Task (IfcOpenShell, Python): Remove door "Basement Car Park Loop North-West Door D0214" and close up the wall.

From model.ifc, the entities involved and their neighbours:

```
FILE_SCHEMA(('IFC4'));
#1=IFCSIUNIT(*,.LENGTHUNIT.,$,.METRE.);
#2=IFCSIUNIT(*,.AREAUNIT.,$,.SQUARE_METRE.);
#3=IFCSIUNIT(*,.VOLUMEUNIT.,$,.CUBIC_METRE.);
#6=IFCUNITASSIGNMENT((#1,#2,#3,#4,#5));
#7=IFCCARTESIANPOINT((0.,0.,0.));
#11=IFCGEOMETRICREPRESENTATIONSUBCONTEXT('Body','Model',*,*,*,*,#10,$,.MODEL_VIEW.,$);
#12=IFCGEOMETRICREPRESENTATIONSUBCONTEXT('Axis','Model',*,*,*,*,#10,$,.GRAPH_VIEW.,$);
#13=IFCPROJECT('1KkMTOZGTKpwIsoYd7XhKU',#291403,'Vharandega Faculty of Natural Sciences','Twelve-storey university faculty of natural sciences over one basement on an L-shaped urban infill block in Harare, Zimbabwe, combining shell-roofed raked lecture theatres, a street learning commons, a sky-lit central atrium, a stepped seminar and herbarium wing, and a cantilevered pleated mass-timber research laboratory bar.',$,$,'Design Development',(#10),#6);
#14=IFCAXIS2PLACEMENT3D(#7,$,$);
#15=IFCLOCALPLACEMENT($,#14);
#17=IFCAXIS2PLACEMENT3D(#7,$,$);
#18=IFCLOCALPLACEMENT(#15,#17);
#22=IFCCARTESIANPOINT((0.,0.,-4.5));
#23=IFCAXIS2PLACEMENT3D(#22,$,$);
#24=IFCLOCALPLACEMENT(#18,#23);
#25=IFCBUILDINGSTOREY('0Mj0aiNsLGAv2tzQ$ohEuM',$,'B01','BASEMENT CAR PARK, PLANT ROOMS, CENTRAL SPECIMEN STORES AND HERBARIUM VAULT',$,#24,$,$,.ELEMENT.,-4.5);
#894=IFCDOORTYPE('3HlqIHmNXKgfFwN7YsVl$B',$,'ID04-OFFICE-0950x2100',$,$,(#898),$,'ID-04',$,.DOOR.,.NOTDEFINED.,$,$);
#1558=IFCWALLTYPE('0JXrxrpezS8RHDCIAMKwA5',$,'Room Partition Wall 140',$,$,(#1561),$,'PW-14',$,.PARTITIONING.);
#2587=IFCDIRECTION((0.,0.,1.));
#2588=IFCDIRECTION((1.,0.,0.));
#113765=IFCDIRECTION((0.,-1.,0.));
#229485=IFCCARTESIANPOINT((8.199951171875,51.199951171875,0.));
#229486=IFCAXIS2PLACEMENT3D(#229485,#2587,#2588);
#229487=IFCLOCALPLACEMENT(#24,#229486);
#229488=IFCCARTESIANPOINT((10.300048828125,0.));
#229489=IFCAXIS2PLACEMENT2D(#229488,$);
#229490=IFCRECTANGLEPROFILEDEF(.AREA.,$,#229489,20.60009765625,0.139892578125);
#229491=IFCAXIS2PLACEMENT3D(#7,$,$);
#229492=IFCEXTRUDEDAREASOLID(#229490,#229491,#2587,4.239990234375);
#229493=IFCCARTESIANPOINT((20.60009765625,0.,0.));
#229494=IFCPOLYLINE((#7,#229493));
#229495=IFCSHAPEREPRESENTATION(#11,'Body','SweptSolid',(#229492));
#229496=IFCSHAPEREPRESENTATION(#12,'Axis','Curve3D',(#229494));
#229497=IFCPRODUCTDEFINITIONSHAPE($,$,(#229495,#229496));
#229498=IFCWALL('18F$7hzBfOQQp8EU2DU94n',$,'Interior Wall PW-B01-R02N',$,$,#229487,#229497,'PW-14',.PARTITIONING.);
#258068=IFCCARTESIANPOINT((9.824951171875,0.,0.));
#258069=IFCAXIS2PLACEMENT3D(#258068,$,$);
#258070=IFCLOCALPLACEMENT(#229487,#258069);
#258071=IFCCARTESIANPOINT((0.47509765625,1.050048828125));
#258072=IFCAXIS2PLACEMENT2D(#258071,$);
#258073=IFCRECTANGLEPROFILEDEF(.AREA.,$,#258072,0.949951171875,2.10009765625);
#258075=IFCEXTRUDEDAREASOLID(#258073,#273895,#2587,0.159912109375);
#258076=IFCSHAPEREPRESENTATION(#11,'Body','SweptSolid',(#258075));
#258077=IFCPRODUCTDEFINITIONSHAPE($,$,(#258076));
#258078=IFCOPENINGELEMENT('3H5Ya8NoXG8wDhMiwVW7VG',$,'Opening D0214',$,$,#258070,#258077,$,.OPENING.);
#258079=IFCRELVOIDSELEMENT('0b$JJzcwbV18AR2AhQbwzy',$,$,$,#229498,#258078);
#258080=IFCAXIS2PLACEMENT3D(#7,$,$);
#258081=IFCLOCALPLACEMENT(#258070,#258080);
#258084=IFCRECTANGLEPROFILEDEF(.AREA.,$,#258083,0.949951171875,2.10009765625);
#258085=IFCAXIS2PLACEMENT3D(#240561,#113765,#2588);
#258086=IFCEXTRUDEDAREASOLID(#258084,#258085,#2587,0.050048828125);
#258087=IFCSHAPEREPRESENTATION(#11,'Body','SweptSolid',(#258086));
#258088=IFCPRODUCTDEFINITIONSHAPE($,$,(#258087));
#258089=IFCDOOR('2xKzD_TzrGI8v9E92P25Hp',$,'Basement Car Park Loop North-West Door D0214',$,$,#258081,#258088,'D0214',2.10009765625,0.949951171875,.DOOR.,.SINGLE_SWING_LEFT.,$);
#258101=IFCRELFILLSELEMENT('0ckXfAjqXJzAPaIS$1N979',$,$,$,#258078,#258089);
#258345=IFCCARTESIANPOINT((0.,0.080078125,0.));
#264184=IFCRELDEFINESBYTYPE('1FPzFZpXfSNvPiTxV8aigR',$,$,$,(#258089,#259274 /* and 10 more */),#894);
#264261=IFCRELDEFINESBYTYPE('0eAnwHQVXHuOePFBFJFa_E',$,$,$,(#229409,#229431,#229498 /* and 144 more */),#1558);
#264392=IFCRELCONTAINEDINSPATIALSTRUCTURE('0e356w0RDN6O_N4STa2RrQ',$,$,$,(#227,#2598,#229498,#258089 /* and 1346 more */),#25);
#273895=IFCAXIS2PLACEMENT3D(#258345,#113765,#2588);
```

```python
import ifcopenshell
import ifcopenshell.api.feature
import ifcopenshell.api.root
import ifcopenshell.geom
import ifcopenshell.util.shape

model = ifcopenshell.open("model.ifc")
settings = ifcopenshell.geom.settings()


def volume(element):
    """Net volume in cubic metres, openings subtracted."""
    shape = ifcopenshell.geom.create_shape(settings, element)
    return ifcopenshell.util.shape.get_volume(shape.geometry)


door = model.by_guid("2xKzD_TzrGI8v9E92P25Hp")
opening = door.FillsVoids[0].RelatingOpeningElement
wall = opening.VoidsElements[0].RelatingBuildingElement
before = volume(wall)

ifcopenshell.api.root.remove_product(model, product=door)
ifcopenshell.api.feature.remove_feature(model, feature=opening)

after = volume(wall)

print(f"wall volume {before:.3f} -> {after:.3f} m3")

model.write("model_edited.ifc")
```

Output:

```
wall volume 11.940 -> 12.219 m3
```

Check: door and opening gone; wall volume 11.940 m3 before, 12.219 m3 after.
